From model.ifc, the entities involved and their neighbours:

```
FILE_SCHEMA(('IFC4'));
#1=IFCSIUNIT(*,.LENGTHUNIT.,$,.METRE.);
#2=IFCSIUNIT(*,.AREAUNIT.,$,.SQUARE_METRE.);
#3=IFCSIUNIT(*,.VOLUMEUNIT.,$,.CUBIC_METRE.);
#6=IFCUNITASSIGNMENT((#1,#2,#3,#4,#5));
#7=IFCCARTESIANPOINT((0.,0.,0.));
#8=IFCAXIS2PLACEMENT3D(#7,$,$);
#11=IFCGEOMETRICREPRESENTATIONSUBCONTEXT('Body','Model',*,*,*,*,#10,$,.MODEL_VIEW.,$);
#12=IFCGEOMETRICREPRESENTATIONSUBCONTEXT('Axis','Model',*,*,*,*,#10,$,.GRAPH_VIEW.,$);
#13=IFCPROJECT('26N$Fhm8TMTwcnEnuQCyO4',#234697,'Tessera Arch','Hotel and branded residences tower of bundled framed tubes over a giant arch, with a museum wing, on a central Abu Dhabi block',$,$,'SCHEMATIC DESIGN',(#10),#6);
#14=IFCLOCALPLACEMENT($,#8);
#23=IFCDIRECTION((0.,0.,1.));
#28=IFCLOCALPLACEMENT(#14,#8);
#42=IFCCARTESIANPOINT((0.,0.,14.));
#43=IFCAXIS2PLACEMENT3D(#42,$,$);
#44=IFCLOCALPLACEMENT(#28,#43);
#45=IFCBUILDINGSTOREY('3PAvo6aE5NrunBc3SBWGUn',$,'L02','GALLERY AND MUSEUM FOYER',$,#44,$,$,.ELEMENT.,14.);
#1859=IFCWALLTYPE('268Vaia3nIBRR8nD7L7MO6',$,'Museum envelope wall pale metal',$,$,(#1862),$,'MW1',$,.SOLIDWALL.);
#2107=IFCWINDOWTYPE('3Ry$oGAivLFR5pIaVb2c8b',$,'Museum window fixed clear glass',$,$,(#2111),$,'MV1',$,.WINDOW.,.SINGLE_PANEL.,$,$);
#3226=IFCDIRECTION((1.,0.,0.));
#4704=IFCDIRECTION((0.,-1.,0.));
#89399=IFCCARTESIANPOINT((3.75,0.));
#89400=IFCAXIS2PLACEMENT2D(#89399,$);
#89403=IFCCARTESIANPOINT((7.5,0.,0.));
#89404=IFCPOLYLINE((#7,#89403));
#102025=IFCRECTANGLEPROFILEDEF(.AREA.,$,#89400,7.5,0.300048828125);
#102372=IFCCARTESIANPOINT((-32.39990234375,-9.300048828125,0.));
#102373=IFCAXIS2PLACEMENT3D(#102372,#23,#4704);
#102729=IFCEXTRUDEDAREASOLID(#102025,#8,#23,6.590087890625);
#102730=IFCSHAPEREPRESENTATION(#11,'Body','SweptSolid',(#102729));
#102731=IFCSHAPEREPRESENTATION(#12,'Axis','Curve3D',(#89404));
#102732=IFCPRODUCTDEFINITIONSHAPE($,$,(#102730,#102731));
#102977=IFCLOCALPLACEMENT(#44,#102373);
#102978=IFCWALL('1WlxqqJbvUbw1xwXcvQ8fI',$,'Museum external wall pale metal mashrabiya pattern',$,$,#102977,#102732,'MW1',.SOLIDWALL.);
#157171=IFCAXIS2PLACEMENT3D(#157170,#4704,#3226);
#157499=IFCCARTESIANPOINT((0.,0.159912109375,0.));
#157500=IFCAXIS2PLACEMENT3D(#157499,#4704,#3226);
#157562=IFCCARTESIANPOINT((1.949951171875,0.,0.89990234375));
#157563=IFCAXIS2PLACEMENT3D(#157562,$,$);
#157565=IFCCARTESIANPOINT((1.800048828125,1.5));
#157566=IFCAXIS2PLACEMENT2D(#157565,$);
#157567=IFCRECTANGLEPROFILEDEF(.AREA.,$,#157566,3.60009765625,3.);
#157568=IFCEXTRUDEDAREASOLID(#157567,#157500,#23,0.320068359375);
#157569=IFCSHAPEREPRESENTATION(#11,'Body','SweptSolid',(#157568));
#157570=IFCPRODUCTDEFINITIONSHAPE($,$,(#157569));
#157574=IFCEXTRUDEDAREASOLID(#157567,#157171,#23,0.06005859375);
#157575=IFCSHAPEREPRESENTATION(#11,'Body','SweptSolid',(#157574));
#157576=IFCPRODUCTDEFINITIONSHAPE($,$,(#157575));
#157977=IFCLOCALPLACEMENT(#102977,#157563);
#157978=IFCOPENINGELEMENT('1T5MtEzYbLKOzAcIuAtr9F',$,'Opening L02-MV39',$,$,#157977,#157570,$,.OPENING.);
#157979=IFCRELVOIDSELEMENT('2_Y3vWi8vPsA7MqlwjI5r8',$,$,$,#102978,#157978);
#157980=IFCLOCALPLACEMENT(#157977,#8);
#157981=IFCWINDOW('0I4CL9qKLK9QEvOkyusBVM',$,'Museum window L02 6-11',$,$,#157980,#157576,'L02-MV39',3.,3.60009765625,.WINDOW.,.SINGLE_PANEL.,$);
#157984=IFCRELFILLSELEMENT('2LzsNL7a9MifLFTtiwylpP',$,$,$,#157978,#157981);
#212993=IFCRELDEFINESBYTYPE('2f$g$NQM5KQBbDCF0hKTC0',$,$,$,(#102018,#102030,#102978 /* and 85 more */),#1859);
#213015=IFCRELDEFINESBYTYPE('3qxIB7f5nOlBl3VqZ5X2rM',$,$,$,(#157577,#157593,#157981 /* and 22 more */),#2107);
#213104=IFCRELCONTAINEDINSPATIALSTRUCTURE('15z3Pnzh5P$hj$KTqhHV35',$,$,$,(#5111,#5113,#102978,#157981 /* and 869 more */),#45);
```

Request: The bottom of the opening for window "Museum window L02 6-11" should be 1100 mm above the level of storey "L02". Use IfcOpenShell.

```python
import numpy as np
import ifcopenshell
import ifcopenshell.api.geometry
import ifcopenshell.geom
import ifcopenshell.util.element
import ifcopenshell.util.placement
import ifcopenshell.util.shape
import ifcopenshell.util.unit

model = ifcopenshell.open("model.ifc")
unit_scale = ifcopenshell.util.unit.calculate_unit_scale(model)

window = model.by_guid("0I4CL9qKLK9QEvOkyusBVM")
opening = window.FillsVoids[0].RelatingOpeningElement
storey = ifcopenshell.util.element.get_container(window, ifc_class="IfcBuildingStorey")
level = ifcopenshell.util.placement.get_local_placement(storey.ObjectPlacement)[2, 3]

# The opening's origin need not be at the sill, so measure its lowest point.
shape = ifcopenshell.geom.create_shape(ifcopenshell.geom.settings(), opening)
bottom = ifcopenshell.util.shape.get_shape_bottom_elevation(shape, shape.geometry) / unit_scale
dz = level + 1.1 / unit_scale - bottom

shift = np.array([0.0, 0.0, dz])
# The window is placed relative to its opening, so it follows when the opening moves.
matrix = ifcopenshell.util.placement.get_local_placement(opening.ObjectPlacement)
matrix[:3, 3] += shift
ifcopenshell.api.geometry.edit_object_placement(
    model, product=opening, matrix=matrix, is_si=False, should_transform_children=True
)

print(f"moved by {dz * unit_scale:+.3f} m")

model.write("model_rev.ifc")
```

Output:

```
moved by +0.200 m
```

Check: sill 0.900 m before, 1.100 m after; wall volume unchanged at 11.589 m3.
